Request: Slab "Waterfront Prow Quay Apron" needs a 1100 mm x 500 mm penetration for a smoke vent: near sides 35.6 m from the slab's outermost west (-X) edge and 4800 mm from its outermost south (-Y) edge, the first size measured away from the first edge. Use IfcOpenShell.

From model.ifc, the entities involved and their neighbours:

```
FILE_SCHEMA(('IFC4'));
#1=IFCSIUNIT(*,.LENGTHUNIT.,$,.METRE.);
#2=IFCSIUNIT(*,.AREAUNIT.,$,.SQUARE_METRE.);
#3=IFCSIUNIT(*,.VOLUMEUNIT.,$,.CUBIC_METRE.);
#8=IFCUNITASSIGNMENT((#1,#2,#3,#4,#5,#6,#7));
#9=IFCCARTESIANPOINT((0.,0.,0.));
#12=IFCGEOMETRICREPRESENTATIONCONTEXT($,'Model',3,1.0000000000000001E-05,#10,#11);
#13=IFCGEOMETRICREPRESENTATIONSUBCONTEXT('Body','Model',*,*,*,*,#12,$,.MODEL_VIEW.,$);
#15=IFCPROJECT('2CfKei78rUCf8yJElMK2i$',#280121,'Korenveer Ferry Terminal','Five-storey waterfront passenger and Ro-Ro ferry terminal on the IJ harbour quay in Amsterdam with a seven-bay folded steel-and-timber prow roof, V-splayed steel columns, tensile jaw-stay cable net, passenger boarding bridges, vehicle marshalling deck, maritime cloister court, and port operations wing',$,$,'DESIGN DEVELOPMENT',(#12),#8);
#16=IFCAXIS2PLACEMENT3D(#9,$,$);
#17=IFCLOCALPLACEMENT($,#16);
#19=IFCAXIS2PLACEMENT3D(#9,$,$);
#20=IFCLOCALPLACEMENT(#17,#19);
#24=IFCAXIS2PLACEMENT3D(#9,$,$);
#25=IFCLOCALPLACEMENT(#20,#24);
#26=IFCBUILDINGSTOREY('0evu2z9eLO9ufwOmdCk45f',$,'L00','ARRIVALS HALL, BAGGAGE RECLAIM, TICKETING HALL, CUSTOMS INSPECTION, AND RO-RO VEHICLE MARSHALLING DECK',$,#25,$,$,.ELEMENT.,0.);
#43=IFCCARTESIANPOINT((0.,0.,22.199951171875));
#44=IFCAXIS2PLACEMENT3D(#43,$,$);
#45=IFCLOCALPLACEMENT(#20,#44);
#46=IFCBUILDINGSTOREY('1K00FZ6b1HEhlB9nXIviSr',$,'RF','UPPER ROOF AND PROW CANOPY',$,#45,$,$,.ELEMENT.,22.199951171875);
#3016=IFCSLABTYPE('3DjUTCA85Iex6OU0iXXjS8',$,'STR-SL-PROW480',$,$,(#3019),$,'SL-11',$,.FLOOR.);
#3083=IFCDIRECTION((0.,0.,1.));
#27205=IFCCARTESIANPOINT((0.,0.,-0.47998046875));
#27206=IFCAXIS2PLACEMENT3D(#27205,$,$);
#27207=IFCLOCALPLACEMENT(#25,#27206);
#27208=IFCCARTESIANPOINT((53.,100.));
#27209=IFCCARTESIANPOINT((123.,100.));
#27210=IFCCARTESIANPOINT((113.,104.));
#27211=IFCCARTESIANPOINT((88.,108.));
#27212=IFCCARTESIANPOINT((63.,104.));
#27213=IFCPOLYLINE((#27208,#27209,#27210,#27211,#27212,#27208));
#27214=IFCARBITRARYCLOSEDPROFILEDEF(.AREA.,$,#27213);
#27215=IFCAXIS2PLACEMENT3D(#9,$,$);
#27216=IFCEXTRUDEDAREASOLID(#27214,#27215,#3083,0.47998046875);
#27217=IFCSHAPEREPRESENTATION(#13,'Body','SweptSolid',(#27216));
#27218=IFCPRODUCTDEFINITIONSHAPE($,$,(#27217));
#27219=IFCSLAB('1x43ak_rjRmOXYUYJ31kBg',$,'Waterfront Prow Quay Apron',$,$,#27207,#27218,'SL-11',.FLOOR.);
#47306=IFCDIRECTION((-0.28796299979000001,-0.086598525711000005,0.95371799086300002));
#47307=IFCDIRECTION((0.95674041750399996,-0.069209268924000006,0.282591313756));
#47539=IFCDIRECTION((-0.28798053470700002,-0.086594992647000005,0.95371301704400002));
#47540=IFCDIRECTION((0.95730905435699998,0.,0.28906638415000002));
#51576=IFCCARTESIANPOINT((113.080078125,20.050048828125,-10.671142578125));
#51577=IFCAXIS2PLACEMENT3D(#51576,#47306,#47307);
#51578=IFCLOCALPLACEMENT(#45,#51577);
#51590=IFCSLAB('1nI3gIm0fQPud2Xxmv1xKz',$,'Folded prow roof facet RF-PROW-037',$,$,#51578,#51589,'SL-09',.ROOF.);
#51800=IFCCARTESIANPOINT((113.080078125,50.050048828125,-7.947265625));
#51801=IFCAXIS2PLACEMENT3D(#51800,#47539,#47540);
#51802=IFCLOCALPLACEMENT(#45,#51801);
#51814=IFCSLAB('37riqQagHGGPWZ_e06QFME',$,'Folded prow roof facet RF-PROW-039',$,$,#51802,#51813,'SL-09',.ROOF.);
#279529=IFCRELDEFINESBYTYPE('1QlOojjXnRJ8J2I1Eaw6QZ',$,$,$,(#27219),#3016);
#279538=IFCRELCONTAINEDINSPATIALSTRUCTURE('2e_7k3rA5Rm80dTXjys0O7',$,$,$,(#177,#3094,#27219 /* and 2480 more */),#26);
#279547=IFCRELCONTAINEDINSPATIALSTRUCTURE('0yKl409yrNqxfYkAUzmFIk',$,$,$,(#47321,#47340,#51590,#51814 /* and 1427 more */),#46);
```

```python
import numpy as np
import ifcopenshell
import ifcopenshell.api.feature
import ifcopenshell.api.geometry
import ifcopenshell.api.root
import ifcopenshell.geom
import ifcopenshell.util.placement
import ifcopenshell.util.representation
import ifcopenshell.util.shape
import ifcopenshell.util.unit

model = ifcopenshell.open("model.ifc")
unit_scale = ifcopenshell.util.unit.calculate_unit_scale(model)
settings = ifcopenshell.geom.settings()


def volume(element):
    """Net volume in cubic metres, openings subtracted."""
    shape = ifcopenshell.geom.create_shape(settings, element)
    return ifcopenshell.util.shape.get_volume(shape.geometry)


slab = model.by_guid("1x43ak_rjRmOXYUYJ31kBg")
before = volume(slab)

# Extent in the slab's own axes, in metres. The edges named are its -X and -Y sides.
slab_shape = ifcopenshell.geom.create_shape(settings, slab)
vertices = ifcopenshell.util.shape.get_vertices(slab_shape.geometry)
x_min, y_min, bottom = vertices.min(axis=0)
top = vertices[:, 2].max()

opening = ifcopenshell.api.root.create_entity(model, ifc_class="IfcOpeningElement", name="Smoke vent opening", predefined_type="OPENING")
context = ifcopenshell.util.representation.get_context(model, "Model", "Body", "MODEL_VIEW")
width, depth = 1.1, 0.5
outline = [(0.0, 0.0), (width, 0.0), (width, depth), (0.0, depth), (0.0, 0.0)]
# Overshoot both faces by 50 mm so the cut is clean.
shape = ifcopenshell.api.geometry.add_slab_representation(
    model, context=context, depth=top - bottom + 0.1, polyline=outline
)
ifcopenshell.api.geometry.assign_representation(model, product=opening, representation=shape)

matrix = ifcopenshell.util.placement.get_local_placement(slab.ObjectPlacement)
matrix[:, 3] = matrix @ np.append(np.array([x_min + 35.6, y_min + 4.8, bottom - 0.05]) / unit_scale, 1.0)
ifcopenshell.api.geometry.edit_object_placement(model, product=opening, matrix=matrix, is_si=False)
ifcopenshell.api.feature.add_feature(model, feature=opening, element=slab)

after = volume(slab)

print(f"slab volume {before:.3f} -> {after:.3f} m3")

model.write("model_updated.ifc")
```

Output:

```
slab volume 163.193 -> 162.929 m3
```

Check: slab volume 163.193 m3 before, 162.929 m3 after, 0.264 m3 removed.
